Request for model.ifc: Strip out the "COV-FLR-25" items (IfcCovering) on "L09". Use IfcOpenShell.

First a look at what the model holds.

```python
import ifcopenshell
import ifcopenshell.util.element

model = ifcopenshell.open("model.ifc")
print(model.schema)
storey = next(s for s in model.by_type("IfcBuildingStorey") if s.Name == "L09")
coverings = [e for e in ifcopenshell.util.element.get_decomposition(storey) if e.is_a("IfcCovering")]
seen = {}
for e in coverings:
    element_type = ifcopenshell.util.element.get_type(e)
    name = element_type.Name if element_type not in (None, e) else None
    seen[name] = seen.get(name, 0) + 1
for name, count in sorted(seen.items(), key=str):
    print(count, "x", name)
```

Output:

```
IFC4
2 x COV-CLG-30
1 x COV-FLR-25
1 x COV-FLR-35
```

```python
import ifcopenshell
import ifcopenshell.api.root
import ifcopenshell.util.element

model = ifcopenshell.open("model.ifc")

storey = next(s for s in model.by_type("IfcBuildingStorey") if s.Name == "L09")
coverings = [e for e in ifcopenshell.util.element.get_decomposition(storey) if e.is_a("IfcCovering")]
targets = [e for e in coverings if (t := ifcopenshell.util.element.get_type(e)) not in (None, e) and t.Name == "COV-FLR-25"]

for e in targets:
    ifcopenshell.api.root.remove_product(model, product=e)
print(len(targets), "removed")

model.write("model_v2.ifc")
```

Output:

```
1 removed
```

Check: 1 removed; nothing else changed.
